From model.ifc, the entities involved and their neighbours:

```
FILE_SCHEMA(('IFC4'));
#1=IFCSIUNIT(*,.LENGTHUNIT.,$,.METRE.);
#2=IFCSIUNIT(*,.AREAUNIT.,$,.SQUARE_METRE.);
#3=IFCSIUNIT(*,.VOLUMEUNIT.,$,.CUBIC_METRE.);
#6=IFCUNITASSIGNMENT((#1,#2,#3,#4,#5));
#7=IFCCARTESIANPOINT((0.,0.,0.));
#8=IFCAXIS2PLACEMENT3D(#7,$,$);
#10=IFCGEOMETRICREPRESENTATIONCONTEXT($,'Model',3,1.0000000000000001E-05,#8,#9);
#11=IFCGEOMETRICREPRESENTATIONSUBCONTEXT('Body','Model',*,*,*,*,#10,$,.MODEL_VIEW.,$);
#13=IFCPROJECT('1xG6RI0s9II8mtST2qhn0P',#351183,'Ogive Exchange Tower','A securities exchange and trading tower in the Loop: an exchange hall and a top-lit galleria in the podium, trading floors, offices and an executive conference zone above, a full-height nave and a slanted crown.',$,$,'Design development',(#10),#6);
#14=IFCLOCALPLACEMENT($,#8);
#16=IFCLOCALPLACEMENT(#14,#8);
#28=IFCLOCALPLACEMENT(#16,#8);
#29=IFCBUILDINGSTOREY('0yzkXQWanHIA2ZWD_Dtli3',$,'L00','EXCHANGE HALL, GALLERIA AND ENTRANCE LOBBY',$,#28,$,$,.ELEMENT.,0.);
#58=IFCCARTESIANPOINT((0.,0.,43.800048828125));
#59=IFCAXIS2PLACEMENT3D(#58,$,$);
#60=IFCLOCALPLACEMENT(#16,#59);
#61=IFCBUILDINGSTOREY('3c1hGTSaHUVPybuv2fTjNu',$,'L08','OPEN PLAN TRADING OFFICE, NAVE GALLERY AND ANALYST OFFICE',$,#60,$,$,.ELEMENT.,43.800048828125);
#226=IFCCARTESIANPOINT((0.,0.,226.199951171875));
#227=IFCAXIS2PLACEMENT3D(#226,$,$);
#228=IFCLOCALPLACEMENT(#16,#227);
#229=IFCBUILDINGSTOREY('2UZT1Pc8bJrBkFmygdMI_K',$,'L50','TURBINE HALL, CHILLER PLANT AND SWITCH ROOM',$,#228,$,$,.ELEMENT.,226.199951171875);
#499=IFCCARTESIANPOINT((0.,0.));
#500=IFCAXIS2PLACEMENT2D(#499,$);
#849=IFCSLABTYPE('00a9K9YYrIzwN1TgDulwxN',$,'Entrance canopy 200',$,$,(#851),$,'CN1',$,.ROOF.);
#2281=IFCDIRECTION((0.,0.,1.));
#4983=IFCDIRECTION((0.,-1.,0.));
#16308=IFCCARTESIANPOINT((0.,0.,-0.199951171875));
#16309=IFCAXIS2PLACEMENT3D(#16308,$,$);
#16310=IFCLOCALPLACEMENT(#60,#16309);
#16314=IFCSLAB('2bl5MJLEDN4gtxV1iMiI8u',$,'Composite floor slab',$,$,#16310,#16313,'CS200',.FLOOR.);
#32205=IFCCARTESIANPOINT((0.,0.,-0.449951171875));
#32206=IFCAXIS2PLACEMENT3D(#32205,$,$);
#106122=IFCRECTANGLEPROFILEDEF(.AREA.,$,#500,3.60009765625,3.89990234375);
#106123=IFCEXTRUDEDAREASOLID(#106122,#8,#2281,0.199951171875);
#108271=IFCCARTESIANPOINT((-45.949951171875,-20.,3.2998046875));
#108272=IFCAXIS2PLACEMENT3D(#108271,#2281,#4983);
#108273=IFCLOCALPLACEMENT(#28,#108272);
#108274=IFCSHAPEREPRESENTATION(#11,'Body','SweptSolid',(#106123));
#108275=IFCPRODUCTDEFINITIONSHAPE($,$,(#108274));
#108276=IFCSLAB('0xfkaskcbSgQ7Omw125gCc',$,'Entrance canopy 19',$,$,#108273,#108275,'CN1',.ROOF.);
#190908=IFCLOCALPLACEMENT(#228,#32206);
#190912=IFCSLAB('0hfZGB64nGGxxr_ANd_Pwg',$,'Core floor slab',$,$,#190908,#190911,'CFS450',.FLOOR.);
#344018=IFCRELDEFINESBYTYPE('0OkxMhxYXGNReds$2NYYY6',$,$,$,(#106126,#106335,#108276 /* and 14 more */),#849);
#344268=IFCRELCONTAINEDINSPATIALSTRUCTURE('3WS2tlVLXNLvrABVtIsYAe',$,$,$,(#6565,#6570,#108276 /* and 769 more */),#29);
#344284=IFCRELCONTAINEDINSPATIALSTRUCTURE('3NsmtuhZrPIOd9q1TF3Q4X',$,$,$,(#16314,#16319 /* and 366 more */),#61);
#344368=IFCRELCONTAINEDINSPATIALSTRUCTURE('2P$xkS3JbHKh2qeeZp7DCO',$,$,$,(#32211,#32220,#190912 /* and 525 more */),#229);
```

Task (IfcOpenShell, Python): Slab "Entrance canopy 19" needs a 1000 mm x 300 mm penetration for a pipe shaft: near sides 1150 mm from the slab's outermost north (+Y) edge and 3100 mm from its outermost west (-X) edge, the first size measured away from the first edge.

```python
import numpy as np
import ifcopenshell
import ifcopenshell.api.feature
import ifcopenshell.api.geometry
import ifcopenshell.api.root
import ifcopenshell.geom
import ifcopenshell.util.placement
import ifcopenshell.util.representation
import ifcopenshell.util.shape
import ifcopenshell.util.unit

model = ifcopenshell.open("model.ifc")
unit_scale = ifcopenshell.util.unit.calculate_unit_scale(model)
settings = ifcopenshell.geom.settings()


def volume(element):
    """Net volume in cubic metres, openings subtracted."""
    shape = ifcopenshell.geom.create_shape(settings, element)
    return ifcopenshell.util.shape.get_volume(shape.geometry)


slab = model.by_guid("0xfkaskcbSgQ7Omw125gCc")
before = volume(slab)

# Extent in the slab's own axes, in metres. The edges named are its -X and -Y sides.
slab_shape = ifcopenshell.geom.create_shape(settings, slab)
vertices = ifcopenshell.util.shape.get_vertices(slab_shape.geometry)
x_min, y_min, bottom = vertices.min(axis=0)
top = vertices[:, 2].max()

opening = ifcopenshell.api.root.create_entity(model, ifc_class="IfcOpeningElement", name="Pipe shaft opening", predefined_type="OPENING")
context = ifcopenshell.util.representation.get_context(model, "Model", "Body", "MODEL_VIEW")
width, depth = 1, 0.3
outline = [(0.0, 0.0), (width, 0.0), (width, depth), (0.0, depth), (0.0, 0.0)]
# Overshoot both faces by 50 mm so the cut is clean.
shape = ifcopenshell.api.geometry.add_slab_representation(
    model, context=context, depth=top - bottom + 0.1, polyline=outline
)
ifcopenshell.api.geometry.assign_representation(model, product=opening, representation=shape)

matrix = ifcopenshell.util.placement.get_local_placement(slab.ObjectPlacement)
matrix[:, 3] = matrix @ np.append(np.array([x_min + 1.15, y_min + 3.1, bottom - 0.05]) / unit_scale, 1.0)
ifcopenshell.api.geometry.edit_object_placement(model, product=opening, matrix=matrix, is_si=False)
ifcopenshell.api.feature.add_feature(model, feature=opening, element=slab)

after = volume(slab)

print(f"slab volume {before:.3f} -> {after:.3f} m3")

model.write("model_rev.ifc")
```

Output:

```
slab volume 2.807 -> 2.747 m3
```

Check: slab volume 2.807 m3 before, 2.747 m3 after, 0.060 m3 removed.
